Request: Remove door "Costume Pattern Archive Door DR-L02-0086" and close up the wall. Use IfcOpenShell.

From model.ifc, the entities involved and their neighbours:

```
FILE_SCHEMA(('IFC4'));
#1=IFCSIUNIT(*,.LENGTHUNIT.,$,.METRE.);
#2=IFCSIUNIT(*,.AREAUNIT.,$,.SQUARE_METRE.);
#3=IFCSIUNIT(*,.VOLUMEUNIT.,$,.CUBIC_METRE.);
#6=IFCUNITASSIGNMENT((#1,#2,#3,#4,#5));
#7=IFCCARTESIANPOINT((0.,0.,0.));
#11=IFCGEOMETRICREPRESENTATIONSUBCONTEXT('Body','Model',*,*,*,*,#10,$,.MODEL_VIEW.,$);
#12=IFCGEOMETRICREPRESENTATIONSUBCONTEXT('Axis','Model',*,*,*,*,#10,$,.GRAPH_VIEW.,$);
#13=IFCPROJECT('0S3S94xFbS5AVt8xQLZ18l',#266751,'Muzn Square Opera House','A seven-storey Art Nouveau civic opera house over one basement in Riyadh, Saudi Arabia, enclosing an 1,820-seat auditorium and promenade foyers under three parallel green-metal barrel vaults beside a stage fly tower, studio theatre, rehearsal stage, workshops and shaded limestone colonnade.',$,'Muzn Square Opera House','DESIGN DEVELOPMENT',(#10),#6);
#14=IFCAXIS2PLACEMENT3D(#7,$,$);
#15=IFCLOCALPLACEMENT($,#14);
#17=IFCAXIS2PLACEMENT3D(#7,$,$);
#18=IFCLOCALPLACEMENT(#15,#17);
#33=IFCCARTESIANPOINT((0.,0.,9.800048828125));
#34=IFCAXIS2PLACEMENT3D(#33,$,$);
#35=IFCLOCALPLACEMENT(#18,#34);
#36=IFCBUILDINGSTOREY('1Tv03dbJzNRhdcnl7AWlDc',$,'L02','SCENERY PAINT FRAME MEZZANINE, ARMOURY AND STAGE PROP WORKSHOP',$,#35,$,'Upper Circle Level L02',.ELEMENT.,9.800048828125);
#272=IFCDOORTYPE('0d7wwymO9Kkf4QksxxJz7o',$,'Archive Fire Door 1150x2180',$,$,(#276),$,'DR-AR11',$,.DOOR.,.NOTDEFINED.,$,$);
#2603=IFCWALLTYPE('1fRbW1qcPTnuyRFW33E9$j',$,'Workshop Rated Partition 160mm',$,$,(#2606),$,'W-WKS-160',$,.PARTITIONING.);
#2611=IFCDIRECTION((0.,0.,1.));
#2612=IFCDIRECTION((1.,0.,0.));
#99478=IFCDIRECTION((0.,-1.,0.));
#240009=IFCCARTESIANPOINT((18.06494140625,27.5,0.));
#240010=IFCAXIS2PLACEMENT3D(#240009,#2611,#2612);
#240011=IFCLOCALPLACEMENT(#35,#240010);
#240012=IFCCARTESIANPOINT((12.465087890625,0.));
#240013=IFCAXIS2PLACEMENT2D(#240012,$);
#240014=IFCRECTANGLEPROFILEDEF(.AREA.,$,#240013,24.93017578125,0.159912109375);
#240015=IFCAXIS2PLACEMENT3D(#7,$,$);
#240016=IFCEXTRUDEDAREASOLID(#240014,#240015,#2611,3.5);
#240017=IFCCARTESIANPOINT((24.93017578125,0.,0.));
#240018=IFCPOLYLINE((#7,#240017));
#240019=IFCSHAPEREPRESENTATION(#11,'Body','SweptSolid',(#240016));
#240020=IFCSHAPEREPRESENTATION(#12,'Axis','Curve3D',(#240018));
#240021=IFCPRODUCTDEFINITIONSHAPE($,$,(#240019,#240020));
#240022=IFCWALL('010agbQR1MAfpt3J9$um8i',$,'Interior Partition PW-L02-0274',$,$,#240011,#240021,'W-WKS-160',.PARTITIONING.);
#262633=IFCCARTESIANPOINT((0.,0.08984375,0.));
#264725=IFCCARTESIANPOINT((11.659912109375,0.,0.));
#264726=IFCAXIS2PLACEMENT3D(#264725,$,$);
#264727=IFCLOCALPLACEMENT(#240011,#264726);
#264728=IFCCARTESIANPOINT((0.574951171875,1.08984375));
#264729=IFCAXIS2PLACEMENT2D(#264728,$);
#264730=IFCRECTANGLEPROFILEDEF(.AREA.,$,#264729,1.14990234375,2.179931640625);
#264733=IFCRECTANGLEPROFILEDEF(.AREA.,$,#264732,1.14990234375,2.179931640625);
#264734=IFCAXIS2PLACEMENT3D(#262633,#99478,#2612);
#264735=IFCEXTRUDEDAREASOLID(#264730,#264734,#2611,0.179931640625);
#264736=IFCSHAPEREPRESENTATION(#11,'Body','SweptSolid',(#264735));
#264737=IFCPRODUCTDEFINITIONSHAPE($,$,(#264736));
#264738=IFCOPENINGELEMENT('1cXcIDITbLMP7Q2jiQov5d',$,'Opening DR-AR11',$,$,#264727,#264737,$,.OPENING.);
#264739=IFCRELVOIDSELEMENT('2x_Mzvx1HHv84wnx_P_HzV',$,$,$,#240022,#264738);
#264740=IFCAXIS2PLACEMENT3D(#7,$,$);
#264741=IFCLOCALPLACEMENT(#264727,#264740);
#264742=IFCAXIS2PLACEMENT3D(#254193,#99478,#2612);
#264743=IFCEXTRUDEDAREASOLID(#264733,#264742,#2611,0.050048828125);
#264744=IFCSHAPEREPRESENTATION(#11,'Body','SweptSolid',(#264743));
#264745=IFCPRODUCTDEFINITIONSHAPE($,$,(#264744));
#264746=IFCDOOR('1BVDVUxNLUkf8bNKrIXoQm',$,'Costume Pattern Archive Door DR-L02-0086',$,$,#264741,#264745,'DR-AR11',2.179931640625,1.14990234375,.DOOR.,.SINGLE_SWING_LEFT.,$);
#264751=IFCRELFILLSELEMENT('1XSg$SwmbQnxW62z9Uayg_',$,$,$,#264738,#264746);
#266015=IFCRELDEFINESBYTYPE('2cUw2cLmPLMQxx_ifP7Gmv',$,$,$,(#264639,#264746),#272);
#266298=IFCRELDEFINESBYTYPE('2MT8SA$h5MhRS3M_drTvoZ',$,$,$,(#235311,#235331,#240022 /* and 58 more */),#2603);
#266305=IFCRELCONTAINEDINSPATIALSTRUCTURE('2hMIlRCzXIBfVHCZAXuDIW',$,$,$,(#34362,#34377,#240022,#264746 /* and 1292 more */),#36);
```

```python
import ifcopenshell
import ifcopenshell.api.feature
import ifcopenshell.api.root
import ifcopenshell.geom
import ifcopenshell.util.shape

model = ifcopenshell.open("model.ifc")
settings = ifcopenshell.geom.settings()


def volume(element):
    """Net volume in cubic metres, openings subtracted."""
    shape = ifcopenshell.geom.create_shape(settings, element)
    return ifcopenshell.util.shape.get_volume(shape.geometry)


door = model.by_guid("1BVDVUxNLUkf8bNKrIXoQm")
opening = door.FillsVoids[0].RelatingOpeningElement
wall = opening.VoidsElements[0].RelatingBuildingElement
before = volume(wall)

ifcopenshell.api.root.remove_product(model, product=door)
ifcopenshell.api.feature.remove_feature(model, feature=opening)

after = volume(wall)

print(f"wall volume {before:.3f} -> {after:.3f} m3")

model.write("model-out.ifc")
```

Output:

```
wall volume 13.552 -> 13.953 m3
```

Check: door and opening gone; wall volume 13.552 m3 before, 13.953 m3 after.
